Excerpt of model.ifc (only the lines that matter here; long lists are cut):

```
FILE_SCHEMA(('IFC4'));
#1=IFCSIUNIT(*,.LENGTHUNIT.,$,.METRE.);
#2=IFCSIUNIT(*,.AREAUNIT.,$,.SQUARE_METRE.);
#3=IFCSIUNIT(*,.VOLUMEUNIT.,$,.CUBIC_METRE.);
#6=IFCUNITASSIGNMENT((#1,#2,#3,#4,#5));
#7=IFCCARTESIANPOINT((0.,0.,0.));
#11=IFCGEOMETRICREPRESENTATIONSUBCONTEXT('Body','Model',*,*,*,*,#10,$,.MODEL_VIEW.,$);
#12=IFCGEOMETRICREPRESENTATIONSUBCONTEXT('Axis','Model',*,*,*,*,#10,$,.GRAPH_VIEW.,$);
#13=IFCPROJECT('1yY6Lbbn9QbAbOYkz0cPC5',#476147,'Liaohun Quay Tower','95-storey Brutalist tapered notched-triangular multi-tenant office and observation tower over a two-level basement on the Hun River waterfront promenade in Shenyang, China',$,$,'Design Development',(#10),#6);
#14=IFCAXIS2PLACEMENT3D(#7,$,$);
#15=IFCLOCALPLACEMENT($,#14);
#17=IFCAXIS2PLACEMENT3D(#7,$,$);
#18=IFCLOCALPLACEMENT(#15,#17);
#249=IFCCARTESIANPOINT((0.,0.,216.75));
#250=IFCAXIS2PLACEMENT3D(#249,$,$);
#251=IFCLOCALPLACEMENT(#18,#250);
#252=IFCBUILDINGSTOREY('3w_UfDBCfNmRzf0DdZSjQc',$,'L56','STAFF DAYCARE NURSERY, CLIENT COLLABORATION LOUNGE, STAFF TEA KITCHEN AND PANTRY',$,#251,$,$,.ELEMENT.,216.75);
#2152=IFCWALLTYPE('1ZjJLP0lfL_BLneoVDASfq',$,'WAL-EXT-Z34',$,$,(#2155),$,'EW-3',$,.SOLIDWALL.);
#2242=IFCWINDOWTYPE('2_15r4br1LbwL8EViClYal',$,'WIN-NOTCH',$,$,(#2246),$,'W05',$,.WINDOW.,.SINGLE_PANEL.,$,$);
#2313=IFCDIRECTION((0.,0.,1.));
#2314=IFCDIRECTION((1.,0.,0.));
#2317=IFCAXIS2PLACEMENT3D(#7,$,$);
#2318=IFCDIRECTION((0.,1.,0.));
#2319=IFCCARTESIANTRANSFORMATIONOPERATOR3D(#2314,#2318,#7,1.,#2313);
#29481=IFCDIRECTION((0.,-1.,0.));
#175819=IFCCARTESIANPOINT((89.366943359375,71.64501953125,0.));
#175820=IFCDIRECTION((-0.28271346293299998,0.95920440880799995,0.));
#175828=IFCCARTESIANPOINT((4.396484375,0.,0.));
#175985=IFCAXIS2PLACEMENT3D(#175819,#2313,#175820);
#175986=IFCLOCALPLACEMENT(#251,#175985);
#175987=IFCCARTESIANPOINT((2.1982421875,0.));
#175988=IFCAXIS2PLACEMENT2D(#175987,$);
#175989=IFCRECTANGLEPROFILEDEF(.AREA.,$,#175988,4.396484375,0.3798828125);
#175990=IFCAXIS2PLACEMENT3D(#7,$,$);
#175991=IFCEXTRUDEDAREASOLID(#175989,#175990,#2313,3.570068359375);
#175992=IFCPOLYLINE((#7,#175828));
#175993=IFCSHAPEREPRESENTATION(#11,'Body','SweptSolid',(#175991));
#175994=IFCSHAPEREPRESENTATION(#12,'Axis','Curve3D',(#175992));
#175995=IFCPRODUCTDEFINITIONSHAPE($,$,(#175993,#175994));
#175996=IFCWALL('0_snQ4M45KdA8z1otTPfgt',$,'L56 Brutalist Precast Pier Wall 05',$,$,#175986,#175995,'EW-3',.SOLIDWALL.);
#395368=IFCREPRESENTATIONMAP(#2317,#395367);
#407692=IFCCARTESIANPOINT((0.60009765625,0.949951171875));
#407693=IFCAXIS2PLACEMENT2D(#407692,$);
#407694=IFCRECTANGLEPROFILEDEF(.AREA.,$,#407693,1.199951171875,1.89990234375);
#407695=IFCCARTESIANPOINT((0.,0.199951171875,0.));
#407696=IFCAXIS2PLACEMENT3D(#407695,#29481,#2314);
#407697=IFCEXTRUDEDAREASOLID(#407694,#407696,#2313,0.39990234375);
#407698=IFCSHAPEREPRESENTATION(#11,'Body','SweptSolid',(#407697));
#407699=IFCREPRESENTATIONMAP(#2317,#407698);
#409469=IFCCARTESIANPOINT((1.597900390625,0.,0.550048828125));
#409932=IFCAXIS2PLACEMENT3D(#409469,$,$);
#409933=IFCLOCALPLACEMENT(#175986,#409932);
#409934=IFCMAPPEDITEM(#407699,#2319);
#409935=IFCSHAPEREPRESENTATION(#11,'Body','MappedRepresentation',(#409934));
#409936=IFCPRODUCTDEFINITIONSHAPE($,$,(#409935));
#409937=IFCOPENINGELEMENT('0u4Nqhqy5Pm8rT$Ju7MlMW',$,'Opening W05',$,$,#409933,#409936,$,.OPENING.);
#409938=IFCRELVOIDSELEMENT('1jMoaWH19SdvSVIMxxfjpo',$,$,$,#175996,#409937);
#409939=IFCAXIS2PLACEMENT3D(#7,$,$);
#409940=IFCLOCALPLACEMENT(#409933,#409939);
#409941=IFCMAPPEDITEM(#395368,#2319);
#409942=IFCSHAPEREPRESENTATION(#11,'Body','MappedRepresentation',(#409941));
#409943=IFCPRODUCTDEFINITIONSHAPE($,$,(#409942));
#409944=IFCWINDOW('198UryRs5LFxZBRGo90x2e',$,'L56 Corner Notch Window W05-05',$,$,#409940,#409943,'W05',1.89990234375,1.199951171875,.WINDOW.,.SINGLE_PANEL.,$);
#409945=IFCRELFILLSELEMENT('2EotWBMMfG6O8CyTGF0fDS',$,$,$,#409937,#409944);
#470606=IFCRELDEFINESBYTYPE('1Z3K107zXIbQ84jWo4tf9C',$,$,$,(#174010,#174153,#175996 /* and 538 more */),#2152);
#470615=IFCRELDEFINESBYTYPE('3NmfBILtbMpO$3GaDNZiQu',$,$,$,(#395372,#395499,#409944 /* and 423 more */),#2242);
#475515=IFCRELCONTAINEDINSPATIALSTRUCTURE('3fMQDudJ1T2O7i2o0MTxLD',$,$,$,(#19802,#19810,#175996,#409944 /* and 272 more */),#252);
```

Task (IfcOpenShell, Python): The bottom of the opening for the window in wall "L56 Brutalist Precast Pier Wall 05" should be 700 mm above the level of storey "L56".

```python
import numpy as np
import ifcopenshell
import ifcopenshell.api.geometry
import ifcopenshell.geom
import ifcopenshell.util.element
import ifcopenshell.util.placement
import ifcopenshell.util.shape
import ifcopenshell.util.unit

model = ifcopenshell.open("model.ifc")
unit_scale = ifcopenshell.util.unit.calculate_unit_scale(model)

window = model.by_guid("198UryRs5LFxZBRGo90x2e")
opening = window.FillsVoids[0].RelatingOpeningElement
storey = ifcopenshell.util.element.get_container(window, ifc_class="IfcBuildingStorey")
level = ifcopenshell.util.placement.get_local_placement(storey.ObjectPlacement)[2, 3]

# The opening's origin need not be at the sill, so measure its lowest point.
shape = ifcopenshell.geom.create_shape(ifcopenshell.geom.settings(), opening)
bottom = ifcopenshell.util.shape.get_shape_bottom_elevation(shape, shape.geometry) / unit_scale
dz = level + 0.7 - bottom

shift = np.array([0.0, 0.0, dz])
# The window is placed relative to its opening, so it follows when the opening moves.
matrix = ifcopenshell.util.placement.get_local_placement(opening.ObjectPlacement)
matrix[:3, 3] += shift
ifcopenshell.api.geometry.edit_object_placement(
    model, product=opening, matrix=matrix, is_si=False, should_transform_children=True
)

print(f"moved by {dz * unit_scale:+.3f} m")

model.write("model_updated.ifc")
```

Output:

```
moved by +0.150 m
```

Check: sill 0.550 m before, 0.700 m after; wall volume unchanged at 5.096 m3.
